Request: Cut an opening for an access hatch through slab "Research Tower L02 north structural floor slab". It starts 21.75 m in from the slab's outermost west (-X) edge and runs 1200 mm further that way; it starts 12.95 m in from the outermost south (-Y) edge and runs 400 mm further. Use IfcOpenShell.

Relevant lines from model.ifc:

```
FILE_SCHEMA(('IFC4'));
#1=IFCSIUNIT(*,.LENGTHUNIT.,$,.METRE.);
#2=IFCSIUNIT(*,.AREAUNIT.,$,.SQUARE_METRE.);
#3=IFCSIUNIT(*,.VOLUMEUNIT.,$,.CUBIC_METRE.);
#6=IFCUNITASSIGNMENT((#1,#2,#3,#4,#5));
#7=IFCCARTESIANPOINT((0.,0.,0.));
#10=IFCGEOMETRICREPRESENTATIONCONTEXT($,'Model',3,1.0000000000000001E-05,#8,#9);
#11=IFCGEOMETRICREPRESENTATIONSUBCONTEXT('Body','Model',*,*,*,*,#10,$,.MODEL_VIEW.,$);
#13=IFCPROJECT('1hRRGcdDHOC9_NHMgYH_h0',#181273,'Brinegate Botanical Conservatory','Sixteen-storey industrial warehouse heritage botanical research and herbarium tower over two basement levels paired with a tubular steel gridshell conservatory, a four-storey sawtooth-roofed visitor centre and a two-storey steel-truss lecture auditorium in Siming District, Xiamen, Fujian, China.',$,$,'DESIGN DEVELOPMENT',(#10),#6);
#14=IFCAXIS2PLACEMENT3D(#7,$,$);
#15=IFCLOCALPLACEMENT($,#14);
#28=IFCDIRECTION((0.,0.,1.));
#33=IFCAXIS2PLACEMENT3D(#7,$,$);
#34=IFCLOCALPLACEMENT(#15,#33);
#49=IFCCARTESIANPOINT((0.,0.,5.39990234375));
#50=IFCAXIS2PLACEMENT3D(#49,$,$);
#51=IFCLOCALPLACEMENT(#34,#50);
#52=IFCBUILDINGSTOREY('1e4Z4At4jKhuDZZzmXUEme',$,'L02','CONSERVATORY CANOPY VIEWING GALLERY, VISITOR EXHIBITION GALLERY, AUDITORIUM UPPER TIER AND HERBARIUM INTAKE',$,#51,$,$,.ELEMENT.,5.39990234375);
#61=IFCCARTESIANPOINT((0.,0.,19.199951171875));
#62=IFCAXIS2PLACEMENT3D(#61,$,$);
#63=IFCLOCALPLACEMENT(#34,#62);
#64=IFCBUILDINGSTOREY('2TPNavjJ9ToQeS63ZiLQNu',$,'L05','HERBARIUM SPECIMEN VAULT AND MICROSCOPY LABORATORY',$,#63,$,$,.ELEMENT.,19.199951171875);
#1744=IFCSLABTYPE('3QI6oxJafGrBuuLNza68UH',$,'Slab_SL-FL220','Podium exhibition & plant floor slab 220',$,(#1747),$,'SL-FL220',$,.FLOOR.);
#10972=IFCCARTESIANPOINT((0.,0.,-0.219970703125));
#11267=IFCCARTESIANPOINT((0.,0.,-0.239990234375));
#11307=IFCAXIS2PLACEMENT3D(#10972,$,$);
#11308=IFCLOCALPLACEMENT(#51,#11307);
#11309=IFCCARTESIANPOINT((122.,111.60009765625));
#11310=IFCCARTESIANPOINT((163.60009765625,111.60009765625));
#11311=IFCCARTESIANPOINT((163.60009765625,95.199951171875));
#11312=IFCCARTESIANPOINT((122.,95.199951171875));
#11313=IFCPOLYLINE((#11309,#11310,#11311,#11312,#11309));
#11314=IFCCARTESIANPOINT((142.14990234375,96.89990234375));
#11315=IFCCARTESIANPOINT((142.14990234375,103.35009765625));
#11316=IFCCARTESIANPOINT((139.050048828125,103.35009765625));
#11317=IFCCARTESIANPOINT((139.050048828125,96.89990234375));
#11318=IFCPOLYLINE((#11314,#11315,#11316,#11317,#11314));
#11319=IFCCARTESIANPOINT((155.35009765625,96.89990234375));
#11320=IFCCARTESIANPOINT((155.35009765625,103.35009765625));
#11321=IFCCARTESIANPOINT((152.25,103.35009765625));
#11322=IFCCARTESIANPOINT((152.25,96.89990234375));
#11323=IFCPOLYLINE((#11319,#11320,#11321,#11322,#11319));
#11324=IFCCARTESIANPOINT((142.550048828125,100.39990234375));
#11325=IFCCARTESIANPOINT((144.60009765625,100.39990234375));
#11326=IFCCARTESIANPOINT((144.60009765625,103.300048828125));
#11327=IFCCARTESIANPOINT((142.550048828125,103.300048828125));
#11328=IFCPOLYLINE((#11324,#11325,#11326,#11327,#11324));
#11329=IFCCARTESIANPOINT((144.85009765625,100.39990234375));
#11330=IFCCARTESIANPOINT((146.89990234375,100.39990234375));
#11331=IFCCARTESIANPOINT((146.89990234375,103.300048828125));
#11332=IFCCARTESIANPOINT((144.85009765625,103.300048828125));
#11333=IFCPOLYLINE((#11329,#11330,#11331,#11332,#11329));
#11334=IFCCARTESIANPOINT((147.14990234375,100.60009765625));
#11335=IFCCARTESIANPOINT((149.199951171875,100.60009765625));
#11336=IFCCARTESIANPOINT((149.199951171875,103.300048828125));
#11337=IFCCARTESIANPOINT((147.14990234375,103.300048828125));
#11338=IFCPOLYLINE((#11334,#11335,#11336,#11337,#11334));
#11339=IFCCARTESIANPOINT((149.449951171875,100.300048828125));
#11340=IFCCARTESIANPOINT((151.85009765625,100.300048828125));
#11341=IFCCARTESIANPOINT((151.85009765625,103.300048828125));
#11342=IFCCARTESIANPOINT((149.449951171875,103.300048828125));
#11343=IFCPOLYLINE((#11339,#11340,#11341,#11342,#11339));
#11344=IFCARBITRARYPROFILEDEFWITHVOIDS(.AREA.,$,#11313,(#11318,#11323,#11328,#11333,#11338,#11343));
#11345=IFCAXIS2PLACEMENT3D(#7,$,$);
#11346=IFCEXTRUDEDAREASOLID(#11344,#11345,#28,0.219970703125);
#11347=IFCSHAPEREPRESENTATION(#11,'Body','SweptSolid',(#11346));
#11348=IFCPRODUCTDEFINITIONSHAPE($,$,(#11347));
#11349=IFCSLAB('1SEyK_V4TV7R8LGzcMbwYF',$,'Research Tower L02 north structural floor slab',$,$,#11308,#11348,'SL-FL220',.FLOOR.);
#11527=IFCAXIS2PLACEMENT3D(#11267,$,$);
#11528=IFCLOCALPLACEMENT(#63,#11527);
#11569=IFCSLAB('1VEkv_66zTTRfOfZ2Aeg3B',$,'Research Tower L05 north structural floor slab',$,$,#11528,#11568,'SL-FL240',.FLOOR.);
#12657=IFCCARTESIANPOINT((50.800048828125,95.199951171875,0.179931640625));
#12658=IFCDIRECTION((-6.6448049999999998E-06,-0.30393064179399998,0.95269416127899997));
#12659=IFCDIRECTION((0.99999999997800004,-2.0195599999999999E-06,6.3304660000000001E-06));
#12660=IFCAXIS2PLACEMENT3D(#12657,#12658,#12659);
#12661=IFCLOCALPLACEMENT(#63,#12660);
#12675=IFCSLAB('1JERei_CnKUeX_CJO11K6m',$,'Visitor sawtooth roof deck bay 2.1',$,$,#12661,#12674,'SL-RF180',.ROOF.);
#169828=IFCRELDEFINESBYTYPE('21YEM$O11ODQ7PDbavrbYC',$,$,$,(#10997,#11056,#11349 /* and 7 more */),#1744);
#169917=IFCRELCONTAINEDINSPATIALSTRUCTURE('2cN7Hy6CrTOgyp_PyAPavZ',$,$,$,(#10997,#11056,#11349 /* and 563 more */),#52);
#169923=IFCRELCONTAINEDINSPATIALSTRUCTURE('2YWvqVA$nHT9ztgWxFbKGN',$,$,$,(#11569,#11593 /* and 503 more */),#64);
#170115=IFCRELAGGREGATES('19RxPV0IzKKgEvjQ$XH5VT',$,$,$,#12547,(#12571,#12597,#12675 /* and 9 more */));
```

```python
import numpy as np
import ifcopenshell
import ifcopenshell.api.feature
import ifcopenshell.api.geometry
import ifcopenshell.api.root
import ifcopenshell.geom
import ifcopenshell.util.placement
import ifcopenshell.util.representation
import ifcopenshell.util.shape
import ifcopenshell.util.unit

model = ifcopenshell.open("model.ifc")
unit_scale = ifcopenshell.util.unit.calculate_unit_scale(model)
settings = ifcopenshell.geom.settings()


def volume(element):
    """Net volume in cubic metres, openings subtracted."""
    shape = ifcopenshell.geom.create_shape(settings, element)
    return ifcopenshell.util.shape.get_volume(shape.geometry)


slab = model.by_guid("1SEyK_V4TV7R8LGzcMbwYF")
before = volume(slab)

# Extent in the slab's own axes, in metres. The edges named are its -X and -Y sides.
slab_shape = ifcopenshell.geom.create_shape(settings, slab)
vertices = ifcopenshell.util.shape.get_vertices(slab_shape.geometry)
x_min, y_min, bottom = vertices.min(axis=0)
top = vertices[:, 2].max()

opening = ifcopenshell.api.root.create_entity(model, ifc_class="IfcOpeningElement", name="Access hatch opening", predefined_type="OPENING")
context = ifcopenshell.util.representation.get_context(model, "Model", "Body", "MODEL_VIEW")
width, depth = 1.2, 0.4
outline = [(0.0, 0.0), (width, 0.0), (width, depth), (0.0, depth), (0.0, 0.0)]
# Overshoot both faces by 50 mm so the cut is clean.
shape = ifcopenshell.api.geometry.add_slab_representation(
    model, context=context, depth=top - bottom + 0.1, polyline=outline
)
ifcopenshell.api.geometry.assign_representation(model, product=opening, representation=shape)

matrix = ifcopenshell.util.placement.get_local_placement(slab.ObjectPlacement)
matrix[:, 3] = matrix @ np.append(np.array([x_min + 21.75, y_min + 12.95, bottom - 0.05]) / unit_scale, 1.0)
ifcopenshell.api.geometry.edit_object_placement(model, product=opening, matrix=matrix, is_si=False)
ifcopenshell.api.feature.add_feature(model, feature=opening, element=slab)

after = volume(slab)

print(f"slab volume {before:.3f} -> {after:.3f} m3")

model.write("model-out.ifc")
```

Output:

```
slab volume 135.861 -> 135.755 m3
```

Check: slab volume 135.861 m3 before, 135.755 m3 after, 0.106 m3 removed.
